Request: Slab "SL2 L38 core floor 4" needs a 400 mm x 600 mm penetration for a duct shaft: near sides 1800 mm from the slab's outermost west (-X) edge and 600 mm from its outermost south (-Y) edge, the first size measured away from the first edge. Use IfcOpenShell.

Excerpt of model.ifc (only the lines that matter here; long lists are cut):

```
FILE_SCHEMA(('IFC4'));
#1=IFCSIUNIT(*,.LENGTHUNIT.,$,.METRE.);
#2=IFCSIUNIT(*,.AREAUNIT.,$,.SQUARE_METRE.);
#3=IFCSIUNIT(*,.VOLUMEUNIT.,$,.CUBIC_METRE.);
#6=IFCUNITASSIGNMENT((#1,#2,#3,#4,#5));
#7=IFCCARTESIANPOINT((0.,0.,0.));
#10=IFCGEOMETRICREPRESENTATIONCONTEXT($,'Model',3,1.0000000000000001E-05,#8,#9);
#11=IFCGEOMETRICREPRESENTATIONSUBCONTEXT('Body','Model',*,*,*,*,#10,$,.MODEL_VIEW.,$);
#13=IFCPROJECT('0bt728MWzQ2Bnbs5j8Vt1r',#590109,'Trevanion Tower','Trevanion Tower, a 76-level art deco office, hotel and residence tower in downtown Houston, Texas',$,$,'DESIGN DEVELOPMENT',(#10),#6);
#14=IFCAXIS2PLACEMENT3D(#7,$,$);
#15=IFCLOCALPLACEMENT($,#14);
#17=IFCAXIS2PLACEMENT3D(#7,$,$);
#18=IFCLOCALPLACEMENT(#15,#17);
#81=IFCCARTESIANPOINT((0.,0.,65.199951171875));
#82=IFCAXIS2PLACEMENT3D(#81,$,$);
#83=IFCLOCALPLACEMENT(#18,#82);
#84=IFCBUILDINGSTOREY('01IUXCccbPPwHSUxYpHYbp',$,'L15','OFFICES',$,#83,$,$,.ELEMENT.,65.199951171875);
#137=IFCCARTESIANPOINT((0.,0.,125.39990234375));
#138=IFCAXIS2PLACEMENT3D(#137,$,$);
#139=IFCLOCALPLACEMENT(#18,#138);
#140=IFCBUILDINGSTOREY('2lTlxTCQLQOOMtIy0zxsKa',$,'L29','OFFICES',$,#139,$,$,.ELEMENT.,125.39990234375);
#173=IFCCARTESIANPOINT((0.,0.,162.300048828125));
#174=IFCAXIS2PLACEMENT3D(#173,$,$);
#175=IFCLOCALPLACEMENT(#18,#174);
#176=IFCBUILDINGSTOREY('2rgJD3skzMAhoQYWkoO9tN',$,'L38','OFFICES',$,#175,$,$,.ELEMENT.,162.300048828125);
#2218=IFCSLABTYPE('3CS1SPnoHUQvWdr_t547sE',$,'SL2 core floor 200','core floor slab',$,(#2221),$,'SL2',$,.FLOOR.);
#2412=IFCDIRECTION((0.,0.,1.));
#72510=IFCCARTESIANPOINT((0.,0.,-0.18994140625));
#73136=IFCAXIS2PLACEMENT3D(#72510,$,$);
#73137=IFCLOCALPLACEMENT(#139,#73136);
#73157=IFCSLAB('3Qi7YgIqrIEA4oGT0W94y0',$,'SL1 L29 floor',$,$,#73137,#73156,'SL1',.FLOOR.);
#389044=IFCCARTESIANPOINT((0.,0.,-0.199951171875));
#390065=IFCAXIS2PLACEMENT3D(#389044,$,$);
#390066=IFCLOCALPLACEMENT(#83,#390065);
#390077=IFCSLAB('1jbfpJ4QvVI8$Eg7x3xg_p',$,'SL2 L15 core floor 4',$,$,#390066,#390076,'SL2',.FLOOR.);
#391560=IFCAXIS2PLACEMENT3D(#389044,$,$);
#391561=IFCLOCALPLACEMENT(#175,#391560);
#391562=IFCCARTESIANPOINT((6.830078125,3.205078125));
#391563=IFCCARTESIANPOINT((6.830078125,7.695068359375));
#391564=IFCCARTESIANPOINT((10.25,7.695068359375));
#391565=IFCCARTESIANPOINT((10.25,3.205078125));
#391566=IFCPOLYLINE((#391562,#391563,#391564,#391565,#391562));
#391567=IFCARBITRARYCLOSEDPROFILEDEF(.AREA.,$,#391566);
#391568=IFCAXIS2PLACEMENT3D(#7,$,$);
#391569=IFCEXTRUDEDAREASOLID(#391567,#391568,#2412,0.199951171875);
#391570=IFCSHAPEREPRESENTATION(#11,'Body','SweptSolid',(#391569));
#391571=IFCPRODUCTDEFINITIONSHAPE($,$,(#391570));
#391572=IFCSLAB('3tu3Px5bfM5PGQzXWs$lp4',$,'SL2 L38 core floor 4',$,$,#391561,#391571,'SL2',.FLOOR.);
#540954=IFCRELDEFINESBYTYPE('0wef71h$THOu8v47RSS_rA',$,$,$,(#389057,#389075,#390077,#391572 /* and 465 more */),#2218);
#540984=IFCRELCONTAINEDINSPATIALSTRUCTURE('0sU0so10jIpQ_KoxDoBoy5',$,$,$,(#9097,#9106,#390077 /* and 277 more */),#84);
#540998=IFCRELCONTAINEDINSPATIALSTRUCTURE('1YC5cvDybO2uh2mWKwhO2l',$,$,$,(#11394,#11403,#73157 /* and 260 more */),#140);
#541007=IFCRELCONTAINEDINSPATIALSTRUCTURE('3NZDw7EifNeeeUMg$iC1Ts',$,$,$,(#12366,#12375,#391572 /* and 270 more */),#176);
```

```python
import numpy as np
import ifcopenshell
import ifcopenshell.api.feature
import ifcopenshell.api.geometry
import ifcopenshell.api.root
import ifcopenshell.geom
import ifcopenshell.util.placement
import ifcopenshell.util.representation
import ifcopenshell.util.shape
import ifcopenshell.util.unit

model = ifcopenshell.open("model.ifc")
unit_scale = ifcopenshell.util.unit.calculate_unit_scale(model)
settings = ifcopenshell.geom.settings()


def volume(element):
    """Net volume in cubic metres, openings subtracted."""
    shape = ifcopenshell.geom.create_shape(settings, element)
    return ifcopenshell.util.shape.get_volume(shape.geometry)


slab = model.by_guid("3tu3Px5bfM5PGQzXWs$lp4")
before = volume(slab)

# Extent in the slab's own axes, in metres. The edges named are its -X and -Y sides.
slab_shape = ifcopenshell.geom.create_shape(settings, slab)
vertices = ifcopenshell.util.shape.get_vertices(slab_shape.geometry)
x_min, y_min, bottom = vertices.min(axis=0)
top = vertices[:, 2].max()

opening = ifcopenshell.api.root.create_entity(model, ifc_class="IfcOpeningElement", name="Duct shaft opening", predefined_type="OPENING")
context = ifcopenshell.util.representation.get_context(model, "Model", "Body", "MODEL_VIEW")
width, depth = 0.4, 0.6
outline = [(0.0, 0.0), (width, 0.0), (width, depth), (0.0, depth), (0.0, 0.0)]
# Overshoot both faces by 50 mm so the cut is clean.
shape = ifcopenshell.api.geometry.add_slab_representation(
    model, context=context, depth=top - bottom + 0.1, polyline=outline
)
ifcopenshell.api.geometry.assign_representation(model, product=opening, representation=shape)

matrix = ifcopenshell.util.placement.get_local_placement(slab.ObjectPlacement)
matrix[:, 3] = matrix @ np.append(np.array([x_min + 1.8, y_min + 0.6, bottom - 0.05]) / unit_scale, 1.0)
ifcopenshell.api.geometry.edit_object_placement(model, product=opening, matrix=matrix, is_si=False)
ifcopenshell.api.feature.add_feature(model, feature=opening, element=slab)

after = volume(slab)

print(f"slab volume {before:.3f} -> {after:.3f} m3")

model.write("model_rev.ifc")
```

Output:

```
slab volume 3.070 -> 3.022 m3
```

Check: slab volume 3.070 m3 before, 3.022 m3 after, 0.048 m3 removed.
